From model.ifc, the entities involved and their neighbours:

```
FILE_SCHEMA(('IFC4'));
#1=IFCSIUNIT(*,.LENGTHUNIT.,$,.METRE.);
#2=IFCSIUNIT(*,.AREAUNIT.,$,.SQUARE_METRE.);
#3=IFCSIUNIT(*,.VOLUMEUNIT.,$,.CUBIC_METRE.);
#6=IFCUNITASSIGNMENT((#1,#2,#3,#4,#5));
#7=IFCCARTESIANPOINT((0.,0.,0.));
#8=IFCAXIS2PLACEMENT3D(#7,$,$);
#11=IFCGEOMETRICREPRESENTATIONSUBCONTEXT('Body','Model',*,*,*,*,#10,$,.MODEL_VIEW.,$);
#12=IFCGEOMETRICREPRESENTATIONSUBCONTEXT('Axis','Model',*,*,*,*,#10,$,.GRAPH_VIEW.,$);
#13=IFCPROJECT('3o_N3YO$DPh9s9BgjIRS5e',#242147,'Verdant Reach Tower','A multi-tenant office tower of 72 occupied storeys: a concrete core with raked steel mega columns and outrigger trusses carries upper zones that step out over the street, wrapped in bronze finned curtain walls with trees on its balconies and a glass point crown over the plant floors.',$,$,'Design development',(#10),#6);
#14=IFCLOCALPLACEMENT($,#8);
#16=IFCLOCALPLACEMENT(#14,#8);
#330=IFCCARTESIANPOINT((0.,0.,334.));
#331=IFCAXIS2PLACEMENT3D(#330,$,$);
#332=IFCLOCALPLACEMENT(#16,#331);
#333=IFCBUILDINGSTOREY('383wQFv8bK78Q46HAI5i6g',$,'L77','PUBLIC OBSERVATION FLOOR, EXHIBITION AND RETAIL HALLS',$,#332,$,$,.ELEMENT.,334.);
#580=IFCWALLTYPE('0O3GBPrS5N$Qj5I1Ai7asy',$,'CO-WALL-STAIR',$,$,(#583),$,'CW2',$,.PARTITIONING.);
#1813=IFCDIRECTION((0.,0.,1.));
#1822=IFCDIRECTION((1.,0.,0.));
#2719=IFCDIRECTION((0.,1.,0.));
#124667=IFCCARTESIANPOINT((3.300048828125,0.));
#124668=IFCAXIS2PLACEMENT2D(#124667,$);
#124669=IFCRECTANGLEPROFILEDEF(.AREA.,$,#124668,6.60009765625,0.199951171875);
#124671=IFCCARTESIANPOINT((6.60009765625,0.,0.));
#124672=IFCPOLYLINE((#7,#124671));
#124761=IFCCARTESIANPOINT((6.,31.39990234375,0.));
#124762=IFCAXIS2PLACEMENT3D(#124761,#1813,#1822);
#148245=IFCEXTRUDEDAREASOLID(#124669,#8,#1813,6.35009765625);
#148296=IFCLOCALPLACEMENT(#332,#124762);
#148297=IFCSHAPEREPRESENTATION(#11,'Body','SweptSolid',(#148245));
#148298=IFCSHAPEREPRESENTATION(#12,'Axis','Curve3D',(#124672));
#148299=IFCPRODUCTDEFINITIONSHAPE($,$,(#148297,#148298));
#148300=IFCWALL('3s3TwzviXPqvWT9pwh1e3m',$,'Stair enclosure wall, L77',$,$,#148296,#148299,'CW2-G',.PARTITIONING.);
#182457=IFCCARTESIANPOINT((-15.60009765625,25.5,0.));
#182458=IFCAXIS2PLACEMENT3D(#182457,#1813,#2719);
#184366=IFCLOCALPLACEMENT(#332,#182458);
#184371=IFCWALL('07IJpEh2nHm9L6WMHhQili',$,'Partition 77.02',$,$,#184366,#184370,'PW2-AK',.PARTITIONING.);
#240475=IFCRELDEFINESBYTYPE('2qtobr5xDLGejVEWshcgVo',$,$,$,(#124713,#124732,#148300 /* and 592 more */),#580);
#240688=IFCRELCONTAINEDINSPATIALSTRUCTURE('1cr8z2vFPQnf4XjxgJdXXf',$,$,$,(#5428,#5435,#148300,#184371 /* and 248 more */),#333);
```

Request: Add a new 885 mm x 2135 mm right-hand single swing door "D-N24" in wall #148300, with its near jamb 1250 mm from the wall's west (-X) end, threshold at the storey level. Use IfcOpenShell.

```python
import numpy as np
import ifcopenshell
import ifcopenshell.api.feature
import ifcopenshell.api.geometry
import ifcopenshell.api.root
import ifcopenshell.api.spatial
import ifcopenshell.geom
import ifcopenshell.util.element
import ifcopenshell.util.placement
import ifcopenshell.util.representation
import ifcopenshell.util.shape
import ifcopenshell.util.unit

model = ifcopenshell.open("model.ifc")
unit_scale = ifcopenshell.util.unit.calculate_unit_scale(model)
settings = ifcopenshell.geom.settings()


def volume(element):
    """Net volume in cubic metres, openings subtracted."""
    shape = ifcopenshell.geom.create_shape(settings, element)
    return ifcopenshell.util.shape.get_volume(shape.geometry)


wall = model.by_guid("3s3TwzviXPqvWT9pwh1e3m")
storey = ifcopenshell.util.element.get_container(wall, ifc_class="IfcBuildingStorey")
context = ifcopenshell.util.representation.get_context(model, "Model", "Body", "MODEL_VIEW")
before = volume(wall)

width, height, from_end, sill = 0.885, 2.135, 1.25, 0.0  # metres

# The wall runs along its own X axis, and the end named is its -X end.
wall_shape = ifcopenshell.geom.create_shape(settings, wall)
x, y, z = ifcopenshell.util.shape.get_vertices(wall_shape.geometry).T
start = x.min() + from_end
face, thickness = float(y.min()), float(y.max() - y.min())
wall_matrix = ifcopenshell.util.placement.get_local_placement(wall.ObjectPlacement)
level = ifcopenshell.util.placement.get_local_placement(storey.ObjectPlacement)[2, 3]


def in_wall(x, y):
    """Placement at x, y metres in the wall's axes, at sill height."""
    matrix = wall_matrix.copy()
    matrix[:, 3] = wall_matrix @ np.array([x / unit_scale, y / unit_scale, 0.0, 1.0])
    matrix[2, 3] = level + sill / unit_scale
    return matrix


# Opening: a box that overshoots both wall faces by 50 mm.
opening = ifcopenshell.api.root.create_entity(model, ifc_class="IfcOpeningElement", predefined_type="OPENING")
box = ifcopenshell.api.geometry.add_wall_representation(
    model, context=context, length=width, height=height, thickness=thickness + 0.1
)
ifcopenshell.api.geometry.assign_representation(model, product=opening, representation=box)
ifcopenshell.api.geometry.edit_object_placement(model, product=opening, matrix=in_wall(start, face - 0.05), is_si=False)
ifcopenshell.api.feature.add_feature(model, feature=opening, element=wall)

door = ifcopenshell.api.root.create_entity(model, ifc_class="IfcDoor", name="D-N24", predefined_type="DOOR")
door.OverallWidth, door.OverallHeight = width / unit_scale, height / unit_scale
door.OperationType = "SINGLE_SWING_RIGHT"
body = ifcopenshell.api.geometry.add_door_representation(
    model,
    context=context,
    overall_width=door.OverallWidth,
    overall_height=door.OverallHeight,
    operation_type="SINGLE_SWING_RIGHT",
    lining_properties={"LiningDepth": thickness / unit_scale, "ThresholdDepth": thickness / unit_scale},
)
ifcopenshell.api.geometry.assign_representation(model, product=door, representation=body)
ifcopenshell.api.spatial.assign_container(model, products=[door], relating_structure=storey)
ifcopenshell.api.feature.add_filling(model, opening=opening, element=door)

# The lining spans the wall, so the door starts at the wall face.
ifcopenshell.api.geometry.edit_object_placement(model, product=door, matrix=in_wall(start, face), is_si=False)

after = volume(wall)

print(f"wall volume {before:.3f} -> {after:.3f} m3")

model.write("model-out.ifc")
```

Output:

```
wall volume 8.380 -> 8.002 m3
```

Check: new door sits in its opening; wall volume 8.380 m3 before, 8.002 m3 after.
